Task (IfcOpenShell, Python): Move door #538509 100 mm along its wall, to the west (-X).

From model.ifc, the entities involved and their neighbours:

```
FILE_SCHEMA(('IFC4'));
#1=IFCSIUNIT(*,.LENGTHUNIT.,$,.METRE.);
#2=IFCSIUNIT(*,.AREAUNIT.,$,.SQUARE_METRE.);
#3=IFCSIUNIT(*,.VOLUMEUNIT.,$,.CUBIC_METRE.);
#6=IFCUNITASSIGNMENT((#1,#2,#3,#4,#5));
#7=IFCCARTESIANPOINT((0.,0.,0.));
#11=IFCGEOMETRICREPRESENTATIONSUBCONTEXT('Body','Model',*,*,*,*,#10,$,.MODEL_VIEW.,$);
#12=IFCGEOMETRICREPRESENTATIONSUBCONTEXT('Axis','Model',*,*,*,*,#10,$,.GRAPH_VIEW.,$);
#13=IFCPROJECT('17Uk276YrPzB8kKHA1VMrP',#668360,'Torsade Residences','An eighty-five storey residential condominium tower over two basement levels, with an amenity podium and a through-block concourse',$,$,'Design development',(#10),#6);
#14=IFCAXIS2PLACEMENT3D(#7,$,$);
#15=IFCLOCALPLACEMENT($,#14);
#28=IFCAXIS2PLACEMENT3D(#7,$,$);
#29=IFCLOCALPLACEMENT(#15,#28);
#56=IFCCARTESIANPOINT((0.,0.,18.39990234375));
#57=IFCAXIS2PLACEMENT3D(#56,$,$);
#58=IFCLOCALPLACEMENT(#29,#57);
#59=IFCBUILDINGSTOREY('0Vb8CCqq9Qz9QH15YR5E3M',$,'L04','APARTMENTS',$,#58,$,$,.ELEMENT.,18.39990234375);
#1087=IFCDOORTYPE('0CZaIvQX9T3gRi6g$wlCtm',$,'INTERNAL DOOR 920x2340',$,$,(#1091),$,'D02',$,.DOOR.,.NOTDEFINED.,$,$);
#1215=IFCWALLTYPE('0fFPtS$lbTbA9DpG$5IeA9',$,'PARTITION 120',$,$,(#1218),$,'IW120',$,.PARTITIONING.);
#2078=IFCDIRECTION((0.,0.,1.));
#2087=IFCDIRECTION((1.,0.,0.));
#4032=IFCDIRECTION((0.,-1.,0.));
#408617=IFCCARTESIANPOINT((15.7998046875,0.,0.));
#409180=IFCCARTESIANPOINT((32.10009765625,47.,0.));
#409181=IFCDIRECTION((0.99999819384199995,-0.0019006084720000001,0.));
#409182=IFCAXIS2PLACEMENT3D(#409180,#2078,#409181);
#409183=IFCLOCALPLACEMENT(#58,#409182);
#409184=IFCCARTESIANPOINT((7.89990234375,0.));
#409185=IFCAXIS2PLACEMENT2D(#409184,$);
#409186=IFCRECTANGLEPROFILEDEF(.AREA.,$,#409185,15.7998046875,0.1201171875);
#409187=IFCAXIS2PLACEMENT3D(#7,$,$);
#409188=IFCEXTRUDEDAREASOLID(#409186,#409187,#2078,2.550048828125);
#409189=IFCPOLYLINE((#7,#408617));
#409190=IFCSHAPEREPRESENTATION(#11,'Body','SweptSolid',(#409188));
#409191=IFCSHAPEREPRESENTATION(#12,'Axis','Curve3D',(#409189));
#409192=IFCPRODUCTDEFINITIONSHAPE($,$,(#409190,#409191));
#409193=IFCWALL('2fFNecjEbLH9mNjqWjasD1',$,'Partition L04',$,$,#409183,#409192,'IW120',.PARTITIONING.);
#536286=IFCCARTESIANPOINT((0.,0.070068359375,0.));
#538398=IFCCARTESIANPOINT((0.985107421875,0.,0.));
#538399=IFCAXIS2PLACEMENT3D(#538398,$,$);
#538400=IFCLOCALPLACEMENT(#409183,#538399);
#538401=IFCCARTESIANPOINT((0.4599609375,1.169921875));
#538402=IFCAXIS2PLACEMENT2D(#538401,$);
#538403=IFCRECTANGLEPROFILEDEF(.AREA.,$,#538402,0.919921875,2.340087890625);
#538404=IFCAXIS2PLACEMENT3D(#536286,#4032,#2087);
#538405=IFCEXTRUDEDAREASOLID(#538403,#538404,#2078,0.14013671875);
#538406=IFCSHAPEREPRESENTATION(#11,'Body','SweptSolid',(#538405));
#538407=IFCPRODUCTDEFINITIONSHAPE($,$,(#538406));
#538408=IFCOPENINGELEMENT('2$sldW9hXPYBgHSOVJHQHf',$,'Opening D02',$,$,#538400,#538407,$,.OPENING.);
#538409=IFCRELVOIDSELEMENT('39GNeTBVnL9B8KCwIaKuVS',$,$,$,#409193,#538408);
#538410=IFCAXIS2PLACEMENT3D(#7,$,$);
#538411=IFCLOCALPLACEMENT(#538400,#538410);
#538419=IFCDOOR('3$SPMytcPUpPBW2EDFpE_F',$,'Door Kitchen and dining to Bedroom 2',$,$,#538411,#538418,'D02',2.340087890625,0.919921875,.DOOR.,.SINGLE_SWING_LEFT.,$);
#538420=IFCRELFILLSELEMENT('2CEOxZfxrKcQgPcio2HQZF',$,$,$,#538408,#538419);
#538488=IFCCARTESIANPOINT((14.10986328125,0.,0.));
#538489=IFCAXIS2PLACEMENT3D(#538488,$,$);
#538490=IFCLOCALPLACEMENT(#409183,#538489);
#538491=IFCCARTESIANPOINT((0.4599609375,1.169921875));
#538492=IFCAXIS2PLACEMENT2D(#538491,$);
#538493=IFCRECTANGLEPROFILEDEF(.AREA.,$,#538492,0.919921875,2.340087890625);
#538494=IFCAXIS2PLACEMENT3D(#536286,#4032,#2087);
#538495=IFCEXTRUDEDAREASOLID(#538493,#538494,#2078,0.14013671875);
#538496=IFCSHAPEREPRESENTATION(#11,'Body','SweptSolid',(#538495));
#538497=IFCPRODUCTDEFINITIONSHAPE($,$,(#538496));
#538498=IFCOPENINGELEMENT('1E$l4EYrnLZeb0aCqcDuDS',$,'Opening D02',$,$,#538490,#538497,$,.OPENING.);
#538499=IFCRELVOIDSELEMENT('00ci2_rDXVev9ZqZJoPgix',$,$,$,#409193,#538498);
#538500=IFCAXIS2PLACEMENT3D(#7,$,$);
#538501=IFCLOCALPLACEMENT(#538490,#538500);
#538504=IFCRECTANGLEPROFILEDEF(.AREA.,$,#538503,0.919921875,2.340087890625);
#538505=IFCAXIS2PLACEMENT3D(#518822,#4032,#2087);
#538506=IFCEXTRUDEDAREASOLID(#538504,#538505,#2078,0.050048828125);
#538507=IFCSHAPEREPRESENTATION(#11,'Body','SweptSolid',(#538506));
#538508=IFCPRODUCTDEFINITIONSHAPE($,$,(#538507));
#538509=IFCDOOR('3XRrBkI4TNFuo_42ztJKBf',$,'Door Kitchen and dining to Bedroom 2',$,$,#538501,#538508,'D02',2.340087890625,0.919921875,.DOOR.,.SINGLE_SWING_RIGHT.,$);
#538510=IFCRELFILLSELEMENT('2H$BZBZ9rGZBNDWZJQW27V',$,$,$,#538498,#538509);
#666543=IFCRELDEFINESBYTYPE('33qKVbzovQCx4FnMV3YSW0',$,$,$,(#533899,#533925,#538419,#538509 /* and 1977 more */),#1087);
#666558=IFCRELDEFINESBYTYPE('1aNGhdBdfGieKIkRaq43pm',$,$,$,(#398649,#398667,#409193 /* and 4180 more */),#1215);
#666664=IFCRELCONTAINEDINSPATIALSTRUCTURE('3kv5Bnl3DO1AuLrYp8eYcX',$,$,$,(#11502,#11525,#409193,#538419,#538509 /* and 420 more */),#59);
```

```python
import ifcopenshell
import ifcopenshell.api.geometry
import ifcopenshell.util.placement

model = ifcopenshell.open("model.ifc")

door = model.by_guid("3XRrBkI4TNFuo_42ztJKBf")
opening = door.FillsVoids[0].RelatingOpeningElement
wall = opening.VoidsElements[0].RelatingBuildingElement

wall_matrix = ifcopenshell.util.placement.get_local_placement(wall.ObjectPlacement)
shift = wall_matrix[:3, 0] * -0.1
before = ifcopenshell.util.placement.get_local_placement(door.ObjectPlacement)[:3, 3].copy()

# The door is placed relative to its opening, so it follows when the opening moves.
matrix = ifcopenshell.util.placement.get_local_placement(opening.ObjectPlacement)
matrix[:3, 3] += shift
ifcopenshell.api.geometry.edit_object_placement(
    model, product=opening, matrix=matrix, is_si=False, should_transform_children=True
)

after = ifcopenshell.util.placement.get_local_placement(door.ObjectPlacement)[:3, 3]
print("door moved by", (after - before).round(3) + 0.0)

model.write("model_updated.ifc")
```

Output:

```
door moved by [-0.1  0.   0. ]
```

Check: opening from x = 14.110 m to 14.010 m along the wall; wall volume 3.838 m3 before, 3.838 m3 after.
